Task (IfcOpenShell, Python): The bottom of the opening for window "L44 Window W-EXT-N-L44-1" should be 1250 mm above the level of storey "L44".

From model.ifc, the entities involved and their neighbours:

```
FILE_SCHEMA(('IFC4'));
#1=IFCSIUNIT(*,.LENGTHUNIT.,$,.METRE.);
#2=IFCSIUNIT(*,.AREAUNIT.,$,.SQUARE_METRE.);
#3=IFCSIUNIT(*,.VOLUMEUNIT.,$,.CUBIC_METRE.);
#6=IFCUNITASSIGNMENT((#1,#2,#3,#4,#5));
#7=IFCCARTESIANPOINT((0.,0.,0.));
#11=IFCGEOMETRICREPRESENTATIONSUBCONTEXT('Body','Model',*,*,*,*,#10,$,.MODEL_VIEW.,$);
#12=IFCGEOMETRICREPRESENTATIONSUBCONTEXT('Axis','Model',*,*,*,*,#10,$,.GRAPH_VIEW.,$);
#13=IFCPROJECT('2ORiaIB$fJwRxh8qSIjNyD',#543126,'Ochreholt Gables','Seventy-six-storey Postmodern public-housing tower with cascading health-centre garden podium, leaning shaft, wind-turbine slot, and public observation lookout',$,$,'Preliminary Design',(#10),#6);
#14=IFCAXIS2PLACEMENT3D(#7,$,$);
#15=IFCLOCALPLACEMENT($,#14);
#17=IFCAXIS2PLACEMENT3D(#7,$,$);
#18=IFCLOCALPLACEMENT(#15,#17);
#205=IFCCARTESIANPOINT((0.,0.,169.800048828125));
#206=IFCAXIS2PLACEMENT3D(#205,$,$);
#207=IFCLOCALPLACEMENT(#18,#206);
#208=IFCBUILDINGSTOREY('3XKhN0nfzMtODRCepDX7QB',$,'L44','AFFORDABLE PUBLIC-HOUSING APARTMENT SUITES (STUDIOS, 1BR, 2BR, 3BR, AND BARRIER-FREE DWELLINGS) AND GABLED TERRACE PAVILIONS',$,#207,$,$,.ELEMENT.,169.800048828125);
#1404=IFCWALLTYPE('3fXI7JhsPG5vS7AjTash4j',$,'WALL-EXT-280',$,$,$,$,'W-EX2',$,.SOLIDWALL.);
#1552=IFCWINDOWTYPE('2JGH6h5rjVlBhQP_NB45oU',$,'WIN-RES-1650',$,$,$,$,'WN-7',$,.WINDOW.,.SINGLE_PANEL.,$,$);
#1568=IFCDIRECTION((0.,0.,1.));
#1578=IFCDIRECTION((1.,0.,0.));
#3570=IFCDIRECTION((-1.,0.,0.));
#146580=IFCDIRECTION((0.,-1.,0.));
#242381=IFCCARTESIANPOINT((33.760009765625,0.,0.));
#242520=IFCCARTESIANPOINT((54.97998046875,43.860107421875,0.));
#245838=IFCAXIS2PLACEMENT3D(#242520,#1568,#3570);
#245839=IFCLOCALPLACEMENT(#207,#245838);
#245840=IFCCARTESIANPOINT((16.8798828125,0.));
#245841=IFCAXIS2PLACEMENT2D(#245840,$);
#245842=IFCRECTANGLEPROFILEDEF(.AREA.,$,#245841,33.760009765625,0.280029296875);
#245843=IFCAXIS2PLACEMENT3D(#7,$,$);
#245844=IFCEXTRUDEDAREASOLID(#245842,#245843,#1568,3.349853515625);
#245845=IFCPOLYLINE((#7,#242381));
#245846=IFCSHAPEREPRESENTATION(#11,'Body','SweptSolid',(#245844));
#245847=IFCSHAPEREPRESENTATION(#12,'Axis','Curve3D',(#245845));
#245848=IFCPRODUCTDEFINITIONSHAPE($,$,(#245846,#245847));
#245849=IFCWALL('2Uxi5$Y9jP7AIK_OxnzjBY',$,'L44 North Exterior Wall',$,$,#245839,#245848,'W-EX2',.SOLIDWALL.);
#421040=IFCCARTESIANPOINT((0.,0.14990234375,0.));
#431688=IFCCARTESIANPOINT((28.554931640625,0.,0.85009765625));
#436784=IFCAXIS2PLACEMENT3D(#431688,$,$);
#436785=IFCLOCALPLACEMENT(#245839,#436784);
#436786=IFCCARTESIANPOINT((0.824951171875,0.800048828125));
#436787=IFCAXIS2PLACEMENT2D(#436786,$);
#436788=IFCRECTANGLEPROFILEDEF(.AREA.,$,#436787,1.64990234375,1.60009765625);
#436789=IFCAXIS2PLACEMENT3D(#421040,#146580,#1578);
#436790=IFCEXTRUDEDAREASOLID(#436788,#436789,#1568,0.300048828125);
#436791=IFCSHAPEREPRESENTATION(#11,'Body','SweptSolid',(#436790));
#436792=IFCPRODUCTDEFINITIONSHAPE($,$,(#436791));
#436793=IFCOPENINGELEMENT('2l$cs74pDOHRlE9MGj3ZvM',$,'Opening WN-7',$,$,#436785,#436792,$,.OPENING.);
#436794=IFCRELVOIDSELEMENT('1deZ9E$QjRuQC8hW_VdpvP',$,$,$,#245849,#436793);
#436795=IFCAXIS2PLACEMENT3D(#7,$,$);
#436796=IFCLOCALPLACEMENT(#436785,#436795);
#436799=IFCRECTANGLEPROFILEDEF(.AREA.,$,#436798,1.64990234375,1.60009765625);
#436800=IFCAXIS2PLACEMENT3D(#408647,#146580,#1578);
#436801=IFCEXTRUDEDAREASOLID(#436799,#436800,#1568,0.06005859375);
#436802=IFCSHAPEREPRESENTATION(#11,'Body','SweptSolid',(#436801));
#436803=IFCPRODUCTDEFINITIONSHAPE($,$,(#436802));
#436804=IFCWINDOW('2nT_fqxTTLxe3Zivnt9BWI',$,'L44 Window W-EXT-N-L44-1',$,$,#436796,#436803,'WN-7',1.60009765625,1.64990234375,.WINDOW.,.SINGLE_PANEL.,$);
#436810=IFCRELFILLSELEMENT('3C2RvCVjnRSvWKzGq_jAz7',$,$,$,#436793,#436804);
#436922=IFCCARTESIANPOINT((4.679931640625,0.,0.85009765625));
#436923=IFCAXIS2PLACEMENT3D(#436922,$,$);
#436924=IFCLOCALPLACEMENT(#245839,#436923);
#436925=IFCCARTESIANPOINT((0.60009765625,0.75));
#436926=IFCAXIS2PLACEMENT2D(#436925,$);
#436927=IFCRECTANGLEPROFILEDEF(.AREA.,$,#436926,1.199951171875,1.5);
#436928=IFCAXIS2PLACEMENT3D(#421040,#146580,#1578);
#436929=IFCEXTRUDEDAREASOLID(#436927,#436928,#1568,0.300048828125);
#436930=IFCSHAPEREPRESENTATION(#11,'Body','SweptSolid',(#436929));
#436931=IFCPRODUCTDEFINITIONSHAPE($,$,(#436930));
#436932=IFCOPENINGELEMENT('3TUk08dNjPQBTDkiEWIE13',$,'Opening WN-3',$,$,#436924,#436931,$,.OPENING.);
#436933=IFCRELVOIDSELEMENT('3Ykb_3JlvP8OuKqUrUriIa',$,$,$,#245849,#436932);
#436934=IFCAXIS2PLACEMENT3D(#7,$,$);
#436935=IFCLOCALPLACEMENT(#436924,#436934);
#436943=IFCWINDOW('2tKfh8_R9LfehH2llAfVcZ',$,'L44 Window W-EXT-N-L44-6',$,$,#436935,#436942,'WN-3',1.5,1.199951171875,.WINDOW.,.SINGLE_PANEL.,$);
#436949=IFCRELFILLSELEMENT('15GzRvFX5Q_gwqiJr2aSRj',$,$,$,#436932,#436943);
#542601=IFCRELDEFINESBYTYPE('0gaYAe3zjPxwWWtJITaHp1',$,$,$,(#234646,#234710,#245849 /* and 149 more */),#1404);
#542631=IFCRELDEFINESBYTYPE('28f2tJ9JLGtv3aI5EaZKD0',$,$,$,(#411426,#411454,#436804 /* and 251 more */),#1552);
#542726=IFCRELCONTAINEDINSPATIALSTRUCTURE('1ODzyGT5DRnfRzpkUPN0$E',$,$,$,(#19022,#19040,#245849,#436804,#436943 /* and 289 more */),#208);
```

```python
import numpy as np
import ifcopenshell
import ifcopenshell.api.geometry
import ifcopenshell.geom
import ifcopenshell.util.element
import ifcopenshell.util.placement
import ifcopenshell.util.shape
import ifcopenshell.util.unit

model = ifcopenshell.open("model.ifc")
unit_scale = ifcopenshell.util.unit.calculate_unit_scale(model)

window = model.by_id(436804)
opening = window.FillsVoids[0].RelatingOpeningElement
storey = ifcopenshell.util.element.get_container(window, ifc_class="IfcBuildingStorey")
level = ifcopenshell.util.placement.get_local_placement(storey.ObjectPlacement)[2, 3]

# The opening's origin need not be at the sill, so measure its lowest point.
shape = ifcopenshell.geom.create_shape(ifcopenshell.geom.settings(), opening)
bottom = ifcopenshell.util.shape.get_shape_bottom_elevation(shape, shape.geometry) / unit_scale
dz = level + 1.25 / unit_scale - bottom

shift = np.array([0.0, 0.0, dz])
# The window is placed relative to its opening, so it follows when the opening moves.
matrix = ifcopenshell.util.placement.get_local_placement(opening.ObjectPlacement)
matrix[:3, 3] += shift
ifcopenshell.api.geometry.edit_object_placement(
    model, product=opening, matrix=matrix, is_si=False, should_transform_children=True
)

print(f"moved by {dz * unit_scale:+.3f} m")

model.write("model_v2.ifc")
```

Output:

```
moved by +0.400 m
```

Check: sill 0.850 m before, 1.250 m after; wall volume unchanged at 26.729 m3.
